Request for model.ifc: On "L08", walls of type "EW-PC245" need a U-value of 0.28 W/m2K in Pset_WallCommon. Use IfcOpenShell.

First a look at what the model holds.

```python
import ifcopenshell
import ifcopenshell.util.element

model = ifcopenshell.open("model.ifc")
print(model.schema)
storey = next(s for s in model.by_type("IfcBuildingStorey") if s.Name == "L08")
walls = [e for e in ifcopenshell.util.element.get_decomposition(storey) if e.is_a("IfcWall")]
seen = {}
for e in walls:
    element_type = ifcopenshell.util.element.get_type(e)
    key = (element_type.Name if element_type != e and element_type else None, ifcopenshell.util.element.get_pset(e, "Pset_WallCommon", "ThermalTransmittance"))
    seen[key] = seen.get(key, 0) + 1
for (name, value), count in sorted(seen.items(), key=str):
    print(count, "x", name, "|", value)
```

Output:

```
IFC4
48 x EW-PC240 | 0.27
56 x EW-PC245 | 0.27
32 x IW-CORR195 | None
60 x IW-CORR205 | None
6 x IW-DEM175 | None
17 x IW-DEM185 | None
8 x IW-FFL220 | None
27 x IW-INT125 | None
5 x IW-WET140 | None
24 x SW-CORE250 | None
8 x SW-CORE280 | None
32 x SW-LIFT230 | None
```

```python
import ifcopenshell
import ifcopenshell.api.pset
import ifcopenshell.util.element

model = ifcopenshell.open("model.ifc")

storey = next(s for s in model.by_type("IfcBuildingStorey") if s.Name == "L08")
walls = [e for e in ifcopenshell.util.element.get_decomposition(storey) if e.is_a("IfcWall")]

count = 0
for e in walls:
    element_type = ifcopenshell.util.element.get_type(e)
    if element_type in (None, e) or element_type.Name != "EW-PC245":
        continue
    # add_pset returns the element's existing set when there is one.
    pset = ifcopenshell.api.pset.add_pset(model, product=e, name="Pset_WallCommon")
    ifcopenshell.api.pset.edit_pset(model, pset=pset, properties={"ThermalTransmittance": 0.28})
    count += 1

print(count, "walls updated")

model.write("model_edited.ifc")
```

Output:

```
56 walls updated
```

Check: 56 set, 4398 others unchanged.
